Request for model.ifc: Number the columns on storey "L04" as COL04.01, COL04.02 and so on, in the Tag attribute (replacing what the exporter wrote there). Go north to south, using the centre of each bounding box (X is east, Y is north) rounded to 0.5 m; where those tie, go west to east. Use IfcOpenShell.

First a look at what the model holds.

```python
import ifcopenshell
import ifcopenshell.util.element
import ifcopenshell.util.placement

model = ifcopenshell.open("model.ifc")
print(model.schema)
storey = next(s for s in model.by_type("IfcBuildingStorey") if s.Name == "L04")
columns = [e for e in ifcopenshell.util.element.get_decomposition(storey) if e.is_a("IfcColumn")]
for e in sorted(columns, key=lambda e: e.id()):
    origin = ifcopenshell.util.placement.get_local_placement(e.ObjectPlacement)[:3, 3]
    print(e.id(), e.Tag, e.Name, origin.round(2) + 0.0, sep=" | ")
```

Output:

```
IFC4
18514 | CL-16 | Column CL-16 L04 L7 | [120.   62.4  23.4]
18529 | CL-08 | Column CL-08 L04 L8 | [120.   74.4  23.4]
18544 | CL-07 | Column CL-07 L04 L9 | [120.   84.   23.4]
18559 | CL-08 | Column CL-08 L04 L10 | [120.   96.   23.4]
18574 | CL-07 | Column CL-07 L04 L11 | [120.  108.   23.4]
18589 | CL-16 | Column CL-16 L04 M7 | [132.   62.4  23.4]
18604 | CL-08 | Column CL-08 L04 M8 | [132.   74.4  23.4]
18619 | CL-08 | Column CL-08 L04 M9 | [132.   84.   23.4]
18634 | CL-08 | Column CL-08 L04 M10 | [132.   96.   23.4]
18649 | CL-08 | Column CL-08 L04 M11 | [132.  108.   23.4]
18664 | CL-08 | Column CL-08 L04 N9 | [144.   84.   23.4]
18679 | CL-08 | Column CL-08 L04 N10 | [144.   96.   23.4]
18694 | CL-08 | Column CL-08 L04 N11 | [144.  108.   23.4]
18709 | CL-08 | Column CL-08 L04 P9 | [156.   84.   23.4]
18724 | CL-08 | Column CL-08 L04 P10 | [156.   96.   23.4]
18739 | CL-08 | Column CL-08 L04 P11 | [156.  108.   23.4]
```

```python
import ifcopenshell
import ifcopenshell.geom
import ifcopenshell.util.element
import ifcopenshell.util.shape

model = ifcopenshell.open("model.ifc")
settings = ifcopenshell.geom.settings()
settings.set("use-world-coords", True)


def centre(element):
    shape = ifcopenshell.geom.create_shape(settings, element)
    return ifcopenshell.util.shape.get_bbox_centroid(shape.geometry)


storey = next(s for s in model.by_type("IfcBuildingStorey") if s.Name == "L04")
columns = [e for e in ifcopenshell.util.element.get_decomposition(storey) if e.is_a("IfcColumn")]

# Insertion points can sit at a corner or the storey origin, so sort by the geometry (in metres).
centres = {e: centre(e) for e in columns}
columns.sort(key=lambda e: (-round(centres[e][1] / 0.5), centres[e][0]))

for i, e in enumerate(columns, start=1):
    number = f"COL04.{i:02d}"
    e.Tag = number
    print(e.id(), number)

model.write("model_updated.ifc")
```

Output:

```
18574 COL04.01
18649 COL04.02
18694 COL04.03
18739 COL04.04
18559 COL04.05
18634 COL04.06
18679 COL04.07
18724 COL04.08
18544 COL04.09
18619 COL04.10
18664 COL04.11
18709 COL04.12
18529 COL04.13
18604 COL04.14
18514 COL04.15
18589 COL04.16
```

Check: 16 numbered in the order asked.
